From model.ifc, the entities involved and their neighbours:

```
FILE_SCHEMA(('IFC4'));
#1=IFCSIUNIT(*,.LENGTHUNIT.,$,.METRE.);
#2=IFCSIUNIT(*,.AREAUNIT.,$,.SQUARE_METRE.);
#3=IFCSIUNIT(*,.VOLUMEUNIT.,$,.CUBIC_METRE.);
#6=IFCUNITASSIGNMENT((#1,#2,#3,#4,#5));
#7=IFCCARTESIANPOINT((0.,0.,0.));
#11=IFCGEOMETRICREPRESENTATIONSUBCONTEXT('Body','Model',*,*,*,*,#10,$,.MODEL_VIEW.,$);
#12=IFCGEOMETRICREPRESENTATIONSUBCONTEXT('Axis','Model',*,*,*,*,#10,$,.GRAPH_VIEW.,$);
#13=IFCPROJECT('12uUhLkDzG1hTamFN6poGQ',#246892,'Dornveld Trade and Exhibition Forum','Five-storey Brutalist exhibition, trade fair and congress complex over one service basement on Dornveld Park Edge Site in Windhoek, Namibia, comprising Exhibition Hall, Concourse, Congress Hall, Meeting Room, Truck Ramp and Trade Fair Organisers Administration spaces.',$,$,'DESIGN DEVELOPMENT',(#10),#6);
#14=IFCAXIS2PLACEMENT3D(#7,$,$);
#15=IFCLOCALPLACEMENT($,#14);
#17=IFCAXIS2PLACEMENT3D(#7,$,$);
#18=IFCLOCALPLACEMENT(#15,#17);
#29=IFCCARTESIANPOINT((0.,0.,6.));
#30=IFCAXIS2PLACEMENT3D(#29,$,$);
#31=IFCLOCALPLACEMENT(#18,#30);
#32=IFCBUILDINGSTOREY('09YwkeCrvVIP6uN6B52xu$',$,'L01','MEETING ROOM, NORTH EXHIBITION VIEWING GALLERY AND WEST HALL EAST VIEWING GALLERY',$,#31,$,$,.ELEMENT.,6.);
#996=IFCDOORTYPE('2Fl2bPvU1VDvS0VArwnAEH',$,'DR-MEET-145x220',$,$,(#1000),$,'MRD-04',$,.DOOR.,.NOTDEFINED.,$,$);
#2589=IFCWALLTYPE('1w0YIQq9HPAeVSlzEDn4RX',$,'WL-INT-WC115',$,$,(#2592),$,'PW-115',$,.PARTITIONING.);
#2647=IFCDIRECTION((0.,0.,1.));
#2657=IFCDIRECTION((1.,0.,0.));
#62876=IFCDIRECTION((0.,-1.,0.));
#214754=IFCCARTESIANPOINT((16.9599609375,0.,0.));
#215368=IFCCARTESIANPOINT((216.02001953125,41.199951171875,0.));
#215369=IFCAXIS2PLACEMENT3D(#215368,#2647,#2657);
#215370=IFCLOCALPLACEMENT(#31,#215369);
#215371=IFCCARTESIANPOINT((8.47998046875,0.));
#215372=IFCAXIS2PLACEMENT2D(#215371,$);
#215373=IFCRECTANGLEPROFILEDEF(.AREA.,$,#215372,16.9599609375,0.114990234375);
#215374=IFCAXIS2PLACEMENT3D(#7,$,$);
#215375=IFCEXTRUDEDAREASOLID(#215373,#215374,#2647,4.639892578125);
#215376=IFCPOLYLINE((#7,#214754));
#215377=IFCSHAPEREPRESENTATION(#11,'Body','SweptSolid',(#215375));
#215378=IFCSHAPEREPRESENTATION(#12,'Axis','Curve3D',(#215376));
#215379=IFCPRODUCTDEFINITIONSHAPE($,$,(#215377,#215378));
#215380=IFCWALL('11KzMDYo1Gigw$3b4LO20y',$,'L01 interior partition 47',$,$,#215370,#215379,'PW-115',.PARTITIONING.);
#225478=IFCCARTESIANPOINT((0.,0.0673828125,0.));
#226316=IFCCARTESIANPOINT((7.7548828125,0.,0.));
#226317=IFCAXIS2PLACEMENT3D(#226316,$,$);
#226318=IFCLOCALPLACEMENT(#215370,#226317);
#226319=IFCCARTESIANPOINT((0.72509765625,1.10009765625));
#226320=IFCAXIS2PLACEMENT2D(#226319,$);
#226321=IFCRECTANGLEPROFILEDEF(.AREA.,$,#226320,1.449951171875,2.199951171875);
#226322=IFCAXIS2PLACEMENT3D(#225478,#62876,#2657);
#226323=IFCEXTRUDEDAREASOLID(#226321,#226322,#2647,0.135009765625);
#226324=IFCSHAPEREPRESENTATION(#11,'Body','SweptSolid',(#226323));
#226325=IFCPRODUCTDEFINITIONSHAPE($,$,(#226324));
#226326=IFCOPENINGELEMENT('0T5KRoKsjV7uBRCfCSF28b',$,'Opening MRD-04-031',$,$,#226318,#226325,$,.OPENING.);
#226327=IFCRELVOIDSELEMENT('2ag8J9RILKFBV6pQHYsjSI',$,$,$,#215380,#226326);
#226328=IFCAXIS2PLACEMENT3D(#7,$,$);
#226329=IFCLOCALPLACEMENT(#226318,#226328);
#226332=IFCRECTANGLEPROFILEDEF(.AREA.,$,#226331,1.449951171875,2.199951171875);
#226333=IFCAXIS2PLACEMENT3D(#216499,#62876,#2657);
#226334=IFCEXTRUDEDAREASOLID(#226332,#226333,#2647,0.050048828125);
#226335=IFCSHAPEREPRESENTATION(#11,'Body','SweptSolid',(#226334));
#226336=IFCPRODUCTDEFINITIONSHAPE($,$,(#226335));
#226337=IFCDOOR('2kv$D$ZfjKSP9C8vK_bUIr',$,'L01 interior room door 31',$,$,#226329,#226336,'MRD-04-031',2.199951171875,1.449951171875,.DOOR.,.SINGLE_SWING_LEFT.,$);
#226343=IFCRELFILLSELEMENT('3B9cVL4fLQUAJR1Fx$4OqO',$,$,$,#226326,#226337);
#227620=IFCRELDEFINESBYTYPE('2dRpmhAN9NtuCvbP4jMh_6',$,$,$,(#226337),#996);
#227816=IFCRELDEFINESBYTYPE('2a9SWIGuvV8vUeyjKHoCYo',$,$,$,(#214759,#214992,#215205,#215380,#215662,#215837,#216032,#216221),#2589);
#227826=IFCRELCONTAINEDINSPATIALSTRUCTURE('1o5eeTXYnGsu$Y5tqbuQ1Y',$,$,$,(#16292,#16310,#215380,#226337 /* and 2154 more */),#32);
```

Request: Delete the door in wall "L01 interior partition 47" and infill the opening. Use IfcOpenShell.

```python
import ifcopenshell
import ifcopenshell.api.feature
import ifcopenshell.api.root
import ifcopenshell.geom
import ifcopenshell.util.shape

model = ifcopenshell.open("model.ifc")
settings = ifcopenshell.geom.settings()


def volume(element):
    """Net volume in cubic metres, openings subtracted."""
    shape = ifcopenshell.geom.create_shape(settings, element)
    return ifcopenshell.util.shape.get_volume(shape.geometry)


door = model.by_guid("2kv$D$ZfjKSP9C8vK_bUIr")
opening = door.FillsVoids[0].RelatingOpeningElement
wall = opening.VoidsElements[0].RelatingBuildingElement
before = volume(wall)

ifcopenshell.api.root.remove_product(model, product=door)
ifcopenshell.api.feature.remove_feature(model, feature=opening)

after = volume(wall)

print(f"wall volume {before:.3f} -> {after:.3f} m3")

model.write("model-out.ifc")
```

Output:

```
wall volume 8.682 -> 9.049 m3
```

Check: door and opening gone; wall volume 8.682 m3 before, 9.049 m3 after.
